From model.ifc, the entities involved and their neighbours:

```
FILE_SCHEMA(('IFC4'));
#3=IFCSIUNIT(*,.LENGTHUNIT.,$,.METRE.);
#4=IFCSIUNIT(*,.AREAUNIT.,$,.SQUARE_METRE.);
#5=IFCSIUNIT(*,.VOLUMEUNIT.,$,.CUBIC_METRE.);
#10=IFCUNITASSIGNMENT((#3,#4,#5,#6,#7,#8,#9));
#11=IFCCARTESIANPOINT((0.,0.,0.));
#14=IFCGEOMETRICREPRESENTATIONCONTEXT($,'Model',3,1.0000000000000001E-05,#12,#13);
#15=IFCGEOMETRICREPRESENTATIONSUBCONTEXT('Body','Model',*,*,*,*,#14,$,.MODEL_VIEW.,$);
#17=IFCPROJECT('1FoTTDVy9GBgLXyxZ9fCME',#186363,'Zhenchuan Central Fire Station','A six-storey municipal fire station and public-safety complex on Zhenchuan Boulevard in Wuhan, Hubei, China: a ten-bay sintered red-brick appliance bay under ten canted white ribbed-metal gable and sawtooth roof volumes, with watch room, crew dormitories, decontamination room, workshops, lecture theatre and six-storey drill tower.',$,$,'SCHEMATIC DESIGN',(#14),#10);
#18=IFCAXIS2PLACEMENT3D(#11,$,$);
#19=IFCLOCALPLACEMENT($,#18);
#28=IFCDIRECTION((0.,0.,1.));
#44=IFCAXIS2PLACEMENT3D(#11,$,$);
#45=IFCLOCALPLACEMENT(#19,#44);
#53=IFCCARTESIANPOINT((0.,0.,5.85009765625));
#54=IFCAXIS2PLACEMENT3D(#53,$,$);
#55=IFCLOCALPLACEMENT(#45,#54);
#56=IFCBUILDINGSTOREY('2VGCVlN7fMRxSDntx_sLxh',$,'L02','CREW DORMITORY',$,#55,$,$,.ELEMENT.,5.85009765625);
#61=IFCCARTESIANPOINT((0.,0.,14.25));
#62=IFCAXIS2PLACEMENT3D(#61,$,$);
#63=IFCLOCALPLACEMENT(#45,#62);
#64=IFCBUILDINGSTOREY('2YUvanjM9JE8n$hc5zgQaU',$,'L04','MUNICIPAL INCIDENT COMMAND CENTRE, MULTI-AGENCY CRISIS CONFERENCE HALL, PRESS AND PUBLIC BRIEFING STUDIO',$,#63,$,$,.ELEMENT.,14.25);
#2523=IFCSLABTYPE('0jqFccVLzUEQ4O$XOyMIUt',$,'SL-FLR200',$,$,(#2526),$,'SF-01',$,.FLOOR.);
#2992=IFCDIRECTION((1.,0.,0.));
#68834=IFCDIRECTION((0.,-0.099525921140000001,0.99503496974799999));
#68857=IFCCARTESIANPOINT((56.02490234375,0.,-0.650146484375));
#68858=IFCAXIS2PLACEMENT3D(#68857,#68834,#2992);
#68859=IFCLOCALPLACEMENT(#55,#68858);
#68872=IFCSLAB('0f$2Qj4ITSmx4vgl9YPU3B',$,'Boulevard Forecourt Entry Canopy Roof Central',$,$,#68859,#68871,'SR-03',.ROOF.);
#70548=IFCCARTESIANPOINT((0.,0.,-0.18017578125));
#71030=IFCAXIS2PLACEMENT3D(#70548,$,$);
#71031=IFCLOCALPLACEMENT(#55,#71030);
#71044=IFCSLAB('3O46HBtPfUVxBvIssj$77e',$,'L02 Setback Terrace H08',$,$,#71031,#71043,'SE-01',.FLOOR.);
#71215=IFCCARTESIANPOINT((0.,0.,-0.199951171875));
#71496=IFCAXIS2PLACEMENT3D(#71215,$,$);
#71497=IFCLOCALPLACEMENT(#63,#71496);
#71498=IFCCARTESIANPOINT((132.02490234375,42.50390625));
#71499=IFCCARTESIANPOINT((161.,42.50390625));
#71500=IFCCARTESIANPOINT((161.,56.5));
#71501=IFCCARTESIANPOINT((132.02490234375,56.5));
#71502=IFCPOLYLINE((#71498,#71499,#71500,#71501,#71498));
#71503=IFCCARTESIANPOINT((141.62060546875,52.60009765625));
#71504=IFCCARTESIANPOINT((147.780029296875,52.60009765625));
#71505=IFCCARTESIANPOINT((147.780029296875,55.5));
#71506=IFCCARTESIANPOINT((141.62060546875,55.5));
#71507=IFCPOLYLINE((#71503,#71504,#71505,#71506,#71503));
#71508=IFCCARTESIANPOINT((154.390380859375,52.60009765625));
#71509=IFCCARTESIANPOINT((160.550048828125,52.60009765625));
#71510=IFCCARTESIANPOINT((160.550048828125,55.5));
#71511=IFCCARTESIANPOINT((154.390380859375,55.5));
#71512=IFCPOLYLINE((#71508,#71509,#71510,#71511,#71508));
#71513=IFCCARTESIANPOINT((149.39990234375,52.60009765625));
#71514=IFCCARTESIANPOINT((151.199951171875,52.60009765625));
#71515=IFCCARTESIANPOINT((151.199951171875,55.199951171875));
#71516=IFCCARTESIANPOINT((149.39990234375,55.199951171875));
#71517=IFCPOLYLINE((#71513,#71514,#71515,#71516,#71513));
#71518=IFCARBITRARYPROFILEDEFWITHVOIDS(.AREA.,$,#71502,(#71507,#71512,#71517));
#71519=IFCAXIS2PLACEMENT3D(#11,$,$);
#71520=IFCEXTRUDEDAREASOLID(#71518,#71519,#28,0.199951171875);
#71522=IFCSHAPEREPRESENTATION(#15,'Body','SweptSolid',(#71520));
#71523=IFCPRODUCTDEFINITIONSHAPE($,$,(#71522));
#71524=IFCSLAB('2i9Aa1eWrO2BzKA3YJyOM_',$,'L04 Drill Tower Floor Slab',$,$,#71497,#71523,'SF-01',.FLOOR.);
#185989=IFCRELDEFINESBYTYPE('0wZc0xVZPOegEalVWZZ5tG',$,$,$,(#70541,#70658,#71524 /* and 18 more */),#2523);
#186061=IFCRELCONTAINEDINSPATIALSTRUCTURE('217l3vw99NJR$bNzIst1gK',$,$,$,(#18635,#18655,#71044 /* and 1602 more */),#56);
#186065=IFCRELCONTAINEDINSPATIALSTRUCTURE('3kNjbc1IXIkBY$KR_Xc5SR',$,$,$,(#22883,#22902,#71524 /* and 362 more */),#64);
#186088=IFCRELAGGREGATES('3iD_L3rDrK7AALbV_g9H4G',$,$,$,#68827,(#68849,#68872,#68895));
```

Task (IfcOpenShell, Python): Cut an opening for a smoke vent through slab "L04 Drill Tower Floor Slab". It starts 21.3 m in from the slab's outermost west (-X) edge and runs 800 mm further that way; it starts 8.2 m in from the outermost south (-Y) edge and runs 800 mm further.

```python
import numpy as np
import ifcopenshell
import ifcopenshell.api.feature
import ifcopenshell.api.geometry
import ifcopenshell.api.root
import ifcopenshell.geom
import ifcopenshell.util.placement
import ifcopenshell.util.representation
import ifcopenshell.util.shape
import ifcopenshell.util.unit

model = ifcopenshell.open("model.ifc")
unit_scale = ifcopenshell.util.unit.calculate_unit_scale(model)
settings = ifcopenshell.geom.settings()


def volume(element):
    """Net volume in cubic metres, openings subtracted."""
    shape = ifcopenshell.geom.create_shape(settings, element)
    return ifcopenshell.util.shape.get_volume(shape.geometry)


slab = model.by_guid("2i9Aa1eWrO2BzKA3YJyOM_")
before = volume(slab)

# Extent in the slab's own axes, in metres. The edges named are its -X and -Y sides.
slab_shape = ifcopenshell.geom.create_shape(settings, slab)
vertices = ifcopenshell.util.shape.get_vertices(slab_shape.geometry)
x_min, y_min, bottom = vertices.min(axis=0)
top = vertices[:, 2].max()

opening = ifcopenshell.api.root.create_entity(model, ifc_class="IfcOpeningElement", name="Smoke vent opening", predefined_type="OPENING")
context = ifcopenshell.util.representation.get_context(model, "Model", "Body", "MODEL_VIEW")
width, depth = 0.8, 0.8
outline = [(0.0, 0.0), (width, 0.0), (width, depth), (0.0, depth), (0.0, 0.0)]
# Overshoot both faces by 50 mm so the cut is clean.
shape = ifcopenshell.api.geometry.add_slab_representation(
    model, context=context, depth=top - bottom + 0.1, polyline=outline
)
ifcopenshell.api.geometry.assign_representation(model, product=opening, representation=shape)

matrix = ifcopenshell.util.placement.get_local_placement(slab.ObjectPlacement)
matrix[:, 3] = matrix @ np.append(np.array([x_min + 21.3, y_min + 8.2, bottom - 0.05]) / unit_scale, 1.0)
ifcopenshell.api.geometry.edit_object_placement(model, product=opening, matrix=matrix, is_si=False)
ifcopenshell.api.feature.add_feature(model, feature=opening, element=slab)

after = volume(slab)

print(f"slab volume {before:.3f} -> {after:.3f} m3")

model.write("model_rev.ifc")
```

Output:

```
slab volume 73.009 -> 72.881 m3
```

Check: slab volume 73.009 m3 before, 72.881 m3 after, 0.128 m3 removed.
